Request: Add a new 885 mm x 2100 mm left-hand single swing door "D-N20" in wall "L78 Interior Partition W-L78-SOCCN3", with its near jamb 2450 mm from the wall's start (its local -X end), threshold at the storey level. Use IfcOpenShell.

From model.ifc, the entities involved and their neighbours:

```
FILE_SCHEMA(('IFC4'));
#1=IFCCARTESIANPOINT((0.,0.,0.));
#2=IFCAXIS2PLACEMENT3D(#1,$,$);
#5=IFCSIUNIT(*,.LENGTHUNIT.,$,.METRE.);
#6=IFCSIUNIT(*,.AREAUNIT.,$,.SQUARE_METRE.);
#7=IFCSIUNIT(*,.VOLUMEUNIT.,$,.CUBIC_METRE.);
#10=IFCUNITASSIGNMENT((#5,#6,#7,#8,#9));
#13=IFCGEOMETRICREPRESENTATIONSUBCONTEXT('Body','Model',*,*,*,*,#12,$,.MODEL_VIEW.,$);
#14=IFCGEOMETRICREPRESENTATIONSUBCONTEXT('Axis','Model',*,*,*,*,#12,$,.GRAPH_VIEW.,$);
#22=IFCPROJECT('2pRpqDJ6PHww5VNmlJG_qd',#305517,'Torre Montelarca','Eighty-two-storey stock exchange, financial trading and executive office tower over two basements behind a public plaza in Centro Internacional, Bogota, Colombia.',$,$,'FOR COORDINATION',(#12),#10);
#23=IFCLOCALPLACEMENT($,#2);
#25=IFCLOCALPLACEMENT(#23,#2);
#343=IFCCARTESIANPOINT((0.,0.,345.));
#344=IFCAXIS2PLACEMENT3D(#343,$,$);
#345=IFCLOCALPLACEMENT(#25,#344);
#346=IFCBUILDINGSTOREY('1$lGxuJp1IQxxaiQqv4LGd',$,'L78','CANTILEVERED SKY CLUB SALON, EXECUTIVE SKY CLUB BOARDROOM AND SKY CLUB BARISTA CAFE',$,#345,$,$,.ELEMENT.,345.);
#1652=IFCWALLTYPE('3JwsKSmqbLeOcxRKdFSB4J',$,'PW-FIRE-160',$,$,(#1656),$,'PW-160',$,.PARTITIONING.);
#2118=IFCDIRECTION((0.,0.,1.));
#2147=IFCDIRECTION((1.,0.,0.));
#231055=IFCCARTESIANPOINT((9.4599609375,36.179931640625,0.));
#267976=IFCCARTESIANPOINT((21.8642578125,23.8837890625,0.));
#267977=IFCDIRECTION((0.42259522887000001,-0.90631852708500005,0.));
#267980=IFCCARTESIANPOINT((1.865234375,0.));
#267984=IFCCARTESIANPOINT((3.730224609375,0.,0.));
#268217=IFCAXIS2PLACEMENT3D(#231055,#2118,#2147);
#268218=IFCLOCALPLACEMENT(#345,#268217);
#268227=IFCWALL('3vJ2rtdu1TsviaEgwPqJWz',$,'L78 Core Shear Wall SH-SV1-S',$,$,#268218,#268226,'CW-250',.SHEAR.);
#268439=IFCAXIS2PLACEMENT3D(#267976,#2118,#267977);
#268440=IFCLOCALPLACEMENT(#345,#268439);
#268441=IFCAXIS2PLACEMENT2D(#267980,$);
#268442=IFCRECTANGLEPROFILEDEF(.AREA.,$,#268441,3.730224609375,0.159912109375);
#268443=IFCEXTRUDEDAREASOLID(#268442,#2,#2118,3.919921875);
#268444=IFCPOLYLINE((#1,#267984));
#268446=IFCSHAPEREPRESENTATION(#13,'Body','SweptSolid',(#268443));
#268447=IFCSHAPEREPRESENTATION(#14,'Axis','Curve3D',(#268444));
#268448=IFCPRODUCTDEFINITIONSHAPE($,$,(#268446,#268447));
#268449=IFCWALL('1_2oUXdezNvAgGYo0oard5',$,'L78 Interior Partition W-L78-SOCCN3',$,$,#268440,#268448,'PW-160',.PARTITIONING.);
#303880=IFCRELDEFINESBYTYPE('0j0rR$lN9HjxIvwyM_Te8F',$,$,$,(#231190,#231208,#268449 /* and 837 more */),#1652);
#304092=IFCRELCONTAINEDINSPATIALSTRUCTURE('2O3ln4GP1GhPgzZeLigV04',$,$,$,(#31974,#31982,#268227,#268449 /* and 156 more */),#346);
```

```python
import numpy as np
import ifcopenshell
import ifcopenshell.api.feature
import ifcopenshell.api.geometry
import ifcopenshell.api.root
import ifcopenshell.api.spatial
import ifcopenshell.geom
import ifcopenshell.util.element
import ifcopenshell.util.placement
import ifcopenshell.util.representation
import ifcopenshell.util.shape
import ifcopenshell.util.unit

model = ifcopenshell.open("model.ifc")
unit_scale = ifcopenshell.util.unit.calculate_unit_scale(model)
settings = ifcopenshell.geom.settings()


def volume(element):
    """Net volume in cubic metres, openings subtracted."""
    shape = ifcopenshell.geom.create_shape(settings, element)
    return ifcopenshell.util.shape.get_volume(shape.geometry)


wall = model.by_guid("1_2oUXdezNvAgGYo0oard5")
storey = ifcopenshell.util.element.get_container(wall, ifc_class="IfcBuildingStorey")
context = ifcopenshell.util.representation.get_context(model, "Model", "Body", "MODEL_VIEW")
before = volume(wall)

width, height, from_end, sill = 0.885, 2.1, 2.45, 0.0  # metres

# The wall runs along its own X axis, and the end named is its -X end.
wall_shape = ifcopenshell.geom.create_shape(settings, wall)
x, y, z = ifcopenshell.util.shape.get_vertices(wall_shape.geometry).T
start = x.min() + from_end
face, thickness = float(y.min()), float(y.max() - y.min())
wall_matrix = ifcopenshell.util.placement.get_local_placement(wall.ObjectPlacement)
level = ifcopenshell.util.placement.get_local_placement(storey.ObjectPlacement)[2, 3]


def in_wall(x, y):
    """Placement at x, y metres in the wall's axes, at sill height."""
    matrix = wall_matrix.copy()
    matrix[:, 3] = wall_matrix @ np.array([x / unit_scale, y / unit_scale, 0.0, 1.0])
    matrix[2, 3] = level + sill / unit_scale
    return matrix


# Opening: a box that overshoots both wall faces by 50 mm.
opening = ifcopenshell.api.root.create_entity(model, ifc_class="IfcOpeningElement", predefined_type="OPENING")
box = ifcopenshell.api.geometry.add_wall_representation(
    model, context=context, length=width, height=height, thickness=thickness + 0.1
)
ifcopenshell.api.geometry.assign_representation(model, product=opening, representation=box)
ifcopenshell.api.geometry.edit_object_placement(model, product=opening, matrix=in_wall(start, face - 0.05), is_si=False)
ifcopenshell.api.feature.add_feature(model, feature=opening, element=wall)

door = ifcopenshell.api.root.create_entity(model, ifc_class="IfcDoor", name="D-N20", predefined_type="DOOR")
door.OverallWidth, door.OverallHeight = width / unit_scale, height / unit_scale
door.OperationType = "SINGLE_SWING_LEFT"
body = ifcopenshell.api.geometry.add_door_representation(
    model,
    context=context,
    overall_width=door.OverallWidth,
    overall_height=door.OverallHeight,
    operation_type="SINGLE_SWING_LEFT",
    lining_properties={"LiningDepth": thickness / unit_scale, "ThresholdDepth": thickness / unit_scale},
)
ifcopenshell.api.geometry.assign_representation(model, product=door, representation=body)
ifcopenshell.api.spatial.assign_container(model, products=[door], relating_structure=storey)
ifcopenshell.api.feature.add_filling(model, opening=opening, element=door)

# The lining spans the wall, so the door starts at the wall face.
ifcopenshell.api.geometry.edit_object_placement(model, product=door, matrix=in_wall(start, face), is_si=False)

after = volume(wall)

print(f"wall volume {before:.3f} -> {after:.3f} m3")

model.write("model_rev.ifc")
```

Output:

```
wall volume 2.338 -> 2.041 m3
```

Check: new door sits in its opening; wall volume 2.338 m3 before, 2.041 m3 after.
